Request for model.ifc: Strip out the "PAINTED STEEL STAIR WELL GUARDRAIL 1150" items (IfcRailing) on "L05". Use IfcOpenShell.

First a look at what the model holds.

```python
import ifcopenshell
import ifcopenshell.util.element

model = ifcopenshell.open("model.ifc")
print(model.schema)
storey = next(s for s in model.by_type("IfcBuildingStorey") if s.Name == "L05")
railings = [e for e in ifcopenshell.util.element.get_decomposition(storey) if e.is_a("IfcRailing")]
seen = {}
for e in railings:
    element_type = ifcopenshell.util.element.get_type(e)
    name = element_type.Name if element_type not in (None, e) else None
    seen[name] = seen.get(name, 0) + 1
for name, count in sorted(seen.items(), key=str):
    print(count, "x", name)
```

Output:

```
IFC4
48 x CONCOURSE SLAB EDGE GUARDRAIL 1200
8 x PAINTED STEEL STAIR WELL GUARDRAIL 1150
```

```python
import ifcopenshell
import ifcopenshell.api.root
import ifcopenshell.util.element

model = ifcopenshell.open("model.ifc")

storey = next(s for s in model.by_type("IfcBuildingStorey") if s.Name == "L05")
railings = [e for e in ifcopenshell.util.element.get_decomposition(storey) if e.is_a("IfcRailing")]
targets = [e for e in railings if (t := ifcopenshell.util.element.get_type(e)) not in (None, e) and t.Name == "PAINTED STEEL STAIR WELL GUARDRAIL 1150"]

for e in targets:
    ifcopenshell.api.root.remove_product(model, product=e)
print(len(targets), "removed")

model.write("model_updated.ifc")
```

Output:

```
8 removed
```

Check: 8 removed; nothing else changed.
